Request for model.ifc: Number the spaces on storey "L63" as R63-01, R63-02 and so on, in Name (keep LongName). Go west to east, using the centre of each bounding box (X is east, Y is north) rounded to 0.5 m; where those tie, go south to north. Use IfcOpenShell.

First a look at what the model holds.

```python
import ifcopenshell
import ifcopenshell.util.element
import ifcopenshell.util.placement

model = ifcopenshell.open("model.ifc")
print(model.schema)
storey = next(s for s in model.by_type("IfcBuildingStorey") if s.Name == "L63")
spaces = [e for e in ifcopenshell.util.element.get_decomposition(storey) if e.is_a("IfcSpace")]
for e in sorted(spaces, key=lambda e: e.id()):
    origin = ifcopenshell.util.placement.get_local_placement(e.ObjectPlacement)[:3, 3]
    print(e.id(), e.Name, e.LongName, origin.round(2) + 0.0, sep=" | ")
```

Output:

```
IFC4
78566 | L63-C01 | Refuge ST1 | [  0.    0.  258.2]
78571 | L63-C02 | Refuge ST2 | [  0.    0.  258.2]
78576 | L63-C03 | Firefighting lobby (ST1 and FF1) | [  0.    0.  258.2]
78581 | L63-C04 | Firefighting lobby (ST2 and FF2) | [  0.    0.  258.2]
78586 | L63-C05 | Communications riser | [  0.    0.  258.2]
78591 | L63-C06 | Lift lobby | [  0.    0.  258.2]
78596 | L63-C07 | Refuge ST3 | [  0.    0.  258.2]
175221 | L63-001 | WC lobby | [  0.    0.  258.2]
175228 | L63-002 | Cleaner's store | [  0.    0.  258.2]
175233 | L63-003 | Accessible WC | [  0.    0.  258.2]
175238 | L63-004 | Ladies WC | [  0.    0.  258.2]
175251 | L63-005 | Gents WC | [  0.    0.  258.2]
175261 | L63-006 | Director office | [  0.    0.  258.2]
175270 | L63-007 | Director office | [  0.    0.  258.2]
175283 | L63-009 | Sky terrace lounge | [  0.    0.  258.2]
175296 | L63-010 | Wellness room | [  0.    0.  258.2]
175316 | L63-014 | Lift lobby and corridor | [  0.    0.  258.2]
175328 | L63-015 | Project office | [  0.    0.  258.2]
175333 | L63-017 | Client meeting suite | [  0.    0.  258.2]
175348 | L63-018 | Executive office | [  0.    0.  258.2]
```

```python
import ifcopenshell
import ifcopenshell.geom
import ifcopenshell.util.element
import ifcopenshell.util.shape

model = ifcopenshell.open("model.ifc")
settings = ifcopenshell.geom.settings()
settings.set("use-world-coords", True)


def centre(element):
    shape = ifcopenshell.geom.create_shape(settings, element)
    return ifcopenshell.util.shape.get_bbox_centroid(shape.geometry)


storey = next(s for s in model.by_type("IfcBuildingStorey") if s.Name == "L63")
spaces = [e for e in ifcopenshell.util.element.get_decomposition(storey) if e.is_a("IfcSpace")]

# Insertion points can sit at a corner or the storey origin, so sort by the geometry (in metres).
centres = {e: centre(e) for e in spaces}
spaces.sort(key=lambda e: (round(centres[e][0] / 0.5), centres[e][1]))

for i, e in enumerate(spaces, start=1):
    number = f"R63-{i:02d}"
    e.Name = number
    print(e.id(), number)

model.write("model-out.ifc")
```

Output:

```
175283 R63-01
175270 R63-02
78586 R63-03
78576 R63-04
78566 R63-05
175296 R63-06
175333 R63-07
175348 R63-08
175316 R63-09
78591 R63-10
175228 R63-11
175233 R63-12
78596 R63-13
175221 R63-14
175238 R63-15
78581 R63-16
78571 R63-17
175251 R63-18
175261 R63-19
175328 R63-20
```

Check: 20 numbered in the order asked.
